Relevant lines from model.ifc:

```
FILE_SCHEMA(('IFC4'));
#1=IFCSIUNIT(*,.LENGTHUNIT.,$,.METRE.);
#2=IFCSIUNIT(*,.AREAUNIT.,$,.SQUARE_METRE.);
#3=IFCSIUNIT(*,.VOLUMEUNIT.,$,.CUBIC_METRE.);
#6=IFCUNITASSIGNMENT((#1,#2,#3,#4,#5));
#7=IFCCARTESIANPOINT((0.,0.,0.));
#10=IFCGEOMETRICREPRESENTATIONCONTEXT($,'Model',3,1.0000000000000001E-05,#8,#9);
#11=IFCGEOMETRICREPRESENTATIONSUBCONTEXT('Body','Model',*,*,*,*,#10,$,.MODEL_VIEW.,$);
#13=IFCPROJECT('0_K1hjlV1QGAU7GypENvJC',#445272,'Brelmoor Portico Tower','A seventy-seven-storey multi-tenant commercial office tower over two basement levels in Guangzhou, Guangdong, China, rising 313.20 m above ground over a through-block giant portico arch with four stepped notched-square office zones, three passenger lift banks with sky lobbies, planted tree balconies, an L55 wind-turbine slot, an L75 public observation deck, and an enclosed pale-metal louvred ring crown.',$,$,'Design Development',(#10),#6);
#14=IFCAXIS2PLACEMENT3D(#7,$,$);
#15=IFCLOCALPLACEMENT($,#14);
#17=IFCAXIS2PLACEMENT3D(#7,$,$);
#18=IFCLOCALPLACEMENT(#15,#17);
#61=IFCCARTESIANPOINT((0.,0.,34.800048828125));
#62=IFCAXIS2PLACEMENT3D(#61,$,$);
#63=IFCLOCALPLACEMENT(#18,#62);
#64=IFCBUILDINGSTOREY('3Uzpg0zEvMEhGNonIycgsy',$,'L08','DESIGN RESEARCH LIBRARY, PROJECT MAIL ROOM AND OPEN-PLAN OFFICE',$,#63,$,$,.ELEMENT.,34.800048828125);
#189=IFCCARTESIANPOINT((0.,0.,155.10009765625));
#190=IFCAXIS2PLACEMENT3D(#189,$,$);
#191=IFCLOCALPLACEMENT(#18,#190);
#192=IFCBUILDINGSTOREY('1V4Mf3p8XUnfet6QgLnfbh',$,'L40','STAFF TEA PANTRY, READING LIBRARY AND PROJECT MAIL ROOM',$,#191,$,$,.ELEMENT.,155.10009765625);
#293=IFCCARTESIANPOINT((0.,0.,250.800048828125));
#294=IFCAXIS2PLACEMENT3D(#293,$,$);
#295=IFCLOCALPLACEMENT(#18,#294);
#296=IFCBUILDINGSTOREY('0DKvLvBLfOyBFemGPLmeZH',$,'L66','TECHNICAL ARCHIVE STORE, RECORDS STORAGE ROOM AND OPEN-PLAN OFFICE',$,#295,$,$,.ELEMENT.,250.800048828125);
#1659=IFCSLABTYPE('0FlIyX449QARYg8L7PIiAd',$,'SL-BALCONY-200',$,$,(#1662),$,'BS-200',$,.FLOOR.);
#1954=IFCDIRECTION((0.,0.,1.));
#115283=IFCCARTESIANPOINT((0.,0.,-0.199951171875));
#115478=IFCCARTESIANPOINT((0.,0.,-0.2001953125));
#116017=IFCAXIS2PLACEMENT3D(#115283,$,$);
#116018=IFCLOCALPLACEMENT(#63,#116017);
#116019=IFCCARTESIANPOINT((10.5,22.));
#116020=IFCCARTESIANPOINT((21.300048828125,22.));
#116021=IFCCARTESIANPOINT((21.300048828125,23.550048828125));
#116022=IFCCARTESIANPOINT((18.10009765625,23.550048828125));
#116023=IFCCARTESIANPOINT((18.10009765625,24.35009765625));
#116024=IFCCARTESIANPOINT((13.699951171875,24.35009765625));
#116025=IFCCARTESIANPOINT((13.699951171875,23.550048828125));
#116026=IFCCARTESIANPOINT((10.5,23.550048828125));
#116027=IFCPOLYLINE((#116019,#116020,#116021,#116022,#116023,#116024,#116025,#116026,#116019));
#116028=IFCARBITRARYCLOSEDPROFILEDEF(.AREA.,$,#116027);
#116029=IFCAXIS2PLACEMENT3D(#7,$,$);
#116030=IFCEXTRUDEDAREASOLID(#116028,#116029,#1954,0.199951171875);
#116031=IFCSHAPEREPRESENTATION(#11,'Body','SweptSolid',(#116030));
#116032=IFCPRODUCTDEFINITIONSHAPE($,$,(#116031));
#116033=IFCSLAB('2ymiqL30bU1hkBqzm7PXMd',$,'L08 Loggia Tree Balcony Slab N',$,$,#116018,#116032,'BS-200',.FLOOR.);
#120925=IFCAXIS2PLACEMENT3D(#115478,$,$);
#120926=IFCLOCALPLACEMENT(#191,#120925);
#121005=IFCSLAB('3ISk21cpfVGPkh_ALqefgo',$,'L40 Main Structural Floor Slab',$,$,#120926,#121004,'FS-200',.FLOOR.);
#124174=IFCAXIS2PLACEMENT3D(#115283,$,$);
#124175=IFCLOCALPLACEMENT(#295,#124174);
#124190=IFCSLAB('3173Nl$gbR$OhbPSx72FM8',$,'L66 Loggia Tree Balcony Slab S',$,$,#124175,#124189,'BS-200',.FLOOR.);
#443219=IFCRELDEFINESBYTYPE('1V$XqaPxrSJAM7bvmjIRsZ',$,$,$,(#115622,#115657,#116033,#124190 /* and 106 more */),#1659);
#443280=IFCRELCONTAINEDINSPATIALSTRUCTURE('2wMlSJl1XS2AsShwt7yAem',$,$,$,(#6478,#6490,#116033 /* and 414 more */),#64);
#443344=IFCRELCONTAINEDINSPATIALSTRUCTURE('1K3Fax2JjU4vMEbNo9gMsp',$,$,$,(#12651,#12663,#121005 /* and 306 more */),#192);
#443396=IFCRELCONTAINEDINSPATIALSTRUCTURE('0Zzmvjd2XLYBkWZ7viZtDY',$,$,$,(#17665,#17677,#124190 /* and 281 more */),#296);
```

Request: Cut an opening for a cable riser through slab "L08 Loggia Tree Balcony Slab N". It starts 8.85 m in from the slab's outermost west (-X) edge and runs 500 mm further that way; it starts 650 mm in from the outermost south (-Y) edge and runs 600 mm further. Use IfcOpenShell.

```python
import numpy as np
import ifcopenshell
import ifcopenshell.api.feature
import ifcopenshell.api.geometry
import ifcopenshell.api.root
import ifcopenshell.geom
import ifcopenshell.util.placement
import ifcopenshell.util.representation
import ifcopenshell.util.shape
import ifcopenshell.util.unit

model = ifcopenshell.open("model.ifc")
unit_scale = ifcopenshell.util.unit.calculate_unit_scale(model)
settings = ifcopenshell.geom.settings()


def volume(element):
    """Net volume in cubic metres, openings subtracted."""
    shape = ifcopenshell.geom.create_shape(settings, element)
    return ifcopenshell.util.shape.get_volume(shape.geometry)


slab = model.by_guid("2ymiqL30bU1hkBqzm7PXMd")
before = volume(slab)

# Extent in the slab's own axes, in metres. The edges named are its -X and -Y sides.
slab_shape = ifcopenshell.geom.create_shape(settings, slab)
vertices = ifcopenshell.util.shape.get_vertices(slab_shape.geometry)
x_min, y_min, bottom = vertices.min(axis=0)
top = vertices[:, 2].max()

opening = ifcopenshell.api.root.create_entity(model, ifc_class="IfcOpeningElement", name="Cable riser opening", predefined_type="OPENING")
context = ifcopenshell.util.representation.get_context(model, "Model", "Body", "MODEL_VIEW")
width, depth = 0.5, 0.6
outline = [(0.0, 0.0), (width, 0.0), (width, depth), (0.0, depth), (0.0, 0.0)]
# Overshoot both faces by 50 mm so the cut is clean.
shape = ifcopenshell.api.geometry.add_slab_representation(
    model, context=context, depth=top - bottom + 0.1, polyline=outline
)
ifcopenshell.api.geometry.assign_representation(model, product=opening, representation=shape)

matrix = ifcopenshell.util.placement.get_local_placement(slab.ObjectPlacement)
matrix[:, 3] = matrix @ np.append(np.array([x_min + 8.85, y_min + 0.65, bottom - 0.05]) / unit_scale, 1.0)
ifcopenshell.api.geometry.edit_object_placement(model, product=opening, matrix=matrix, is_si=False)
ifcopenshell.api.feature.add_feature(model, feature=opening, element=slab)

after = volume(slab)

print(f"slab volume {before:.3f} -> {after:.3f} m3")

model.write("model_rev.ifc")
```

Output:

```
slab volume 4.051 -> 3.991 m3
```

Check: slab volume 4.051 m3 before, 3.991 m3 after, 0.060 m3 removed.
